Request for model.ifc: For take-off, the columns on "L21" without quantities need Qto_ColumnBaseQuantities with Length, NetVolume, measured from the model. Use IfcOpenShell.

First a look at what the model holds.

```python
import ifcopenshell
import ifcopenshell.util.element
import ifcopenshell.util.unit

model = ifcopenshell.open("model.ifc")
print(model.schema)
for unit_type in ("LENGTHUNIT", "AREAUNIT", "VOLUMEUNIT"):
    print(unit_type, ifcopenshell.util.unit.calculate_unit_scale(model, unit_type))
storey = next(s for s in model.by_type("IfcBuildingStorey") if s.Name == "L21")
columns = [e for e in ifcopenshell.util.element.get_decomposition(storey) if e.is_a("IfcColumn")]
for e in sorted(columns, key=lambda e: e.id()):
    print(e.id(), e.is_a(), e.Name, list(ifcopenshell.util.element.get_psets(e, qtos_only=True)), sep=" | ")
```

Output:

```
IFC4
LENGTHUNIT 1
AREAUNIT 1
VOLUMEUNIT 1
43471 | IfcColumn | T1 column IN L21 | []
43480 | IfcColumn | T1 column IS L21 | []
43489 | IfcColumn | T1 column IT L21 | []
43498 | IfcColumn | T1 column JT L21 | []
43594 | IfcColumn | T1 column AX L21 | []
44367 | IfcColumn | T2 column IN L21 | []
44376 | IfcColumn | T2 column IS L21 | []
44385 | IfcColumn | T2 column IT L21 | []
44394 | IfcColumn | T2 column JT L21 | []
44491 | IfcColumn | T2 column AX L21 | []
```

```python
import ifcopenshell
import ifcopenshell.api.pset
import ifcopenshell.geom
import ifcopenshell.util.element
import ifcopenshell.util.shape
import ifcopenshell.util.unit

model = ifcopenshell.open("model.ifc")
unit_scale = ifcopenshell.util.unit.calculate_unit_scale(model)
volume_scale = ifcopenshell.util.unit.calculate_unit_scale(model, "VOLUMEUNIT")
settings = ifcopenshell.geom.settings()

storey = next(s for s in model.by_type("IfcBuildingStorey") if s.Name == "L21")
columns = [e for e in ifcopenshell.util.element.get_decomposition(storey) if e.is_a("IfcColumn")]

for e in sorted(columns, key=lambda e: e.id()):
    if ifcopenshell.util.element.get_psets(e, qtos_only=True, should_inherit=False):
        continue
    # Geometry comes back in metres, in the element's own axes.
    shape = ifcopenshell.geom.create_shape(settings, e)
    values = {
        "Length": ifcopenshell.util.shape.get_z(shape.geometry) / unit_scale,
        "NetVolume": ifcopenshell.util.shape.get_volume(shape.geometry) / volume_scale,
    }
    qto = ifcopenshell.api.pset.add_qto(model, product=e, name="Qto_ColumnBaseQuantities")
    ifcopenshell.api.pset.edit_qto(model, qto=qto, properties=values)
    print(e.id(), {k: round(v, 3) for k, v in values.items()})

model.write("model_updated.ifc")
```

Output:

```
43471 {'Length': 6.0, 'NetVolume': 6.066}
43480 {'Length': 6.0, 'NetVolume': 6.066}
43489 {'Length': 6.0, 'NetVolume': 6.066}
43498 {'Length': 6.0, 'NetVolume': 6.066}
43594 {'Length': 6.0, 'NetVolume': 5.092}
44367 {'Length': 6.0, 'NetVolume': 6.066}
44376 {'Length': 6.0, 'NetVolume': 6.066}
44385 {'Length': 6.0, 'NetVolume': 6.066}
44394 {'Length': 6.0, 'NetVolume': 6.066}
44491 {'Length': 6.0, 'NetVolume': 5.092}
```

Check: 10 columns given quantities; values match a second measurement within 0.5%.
